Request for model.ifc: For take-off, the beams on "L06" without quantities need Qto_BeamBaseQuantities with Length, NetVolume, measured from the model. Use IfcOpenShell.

First a look at what the model holds.

```python
import ifcopenshell
import ifcopenshell.util.element
import ifcopenshell.util.unit

model = ifcopenshell.open("model.ifc")
print(model.schema)
for unit_type in ("LENGTHUNIT", "AREAUNIT", "VOLUMEUNIT"):
    print(unit_type, ifcopenshell.util.unit.calculate_unit_scale(model, unit_type))
storey = next(s for s in model.by_type("IfcBuildingStorey") if s.Name == "L06")
beams = [e for e in ifcopenshell.util.element.get_decomposition(storey) if e.is_a("IfcBeam")]
for e in sorted(beams, key=lambda e: e.id()):
    print(e.id(), e.is_a(), e.Name, list(ifcopenshell.util.element.get_psets(e, qtos_only=True)), sep=" | ")
```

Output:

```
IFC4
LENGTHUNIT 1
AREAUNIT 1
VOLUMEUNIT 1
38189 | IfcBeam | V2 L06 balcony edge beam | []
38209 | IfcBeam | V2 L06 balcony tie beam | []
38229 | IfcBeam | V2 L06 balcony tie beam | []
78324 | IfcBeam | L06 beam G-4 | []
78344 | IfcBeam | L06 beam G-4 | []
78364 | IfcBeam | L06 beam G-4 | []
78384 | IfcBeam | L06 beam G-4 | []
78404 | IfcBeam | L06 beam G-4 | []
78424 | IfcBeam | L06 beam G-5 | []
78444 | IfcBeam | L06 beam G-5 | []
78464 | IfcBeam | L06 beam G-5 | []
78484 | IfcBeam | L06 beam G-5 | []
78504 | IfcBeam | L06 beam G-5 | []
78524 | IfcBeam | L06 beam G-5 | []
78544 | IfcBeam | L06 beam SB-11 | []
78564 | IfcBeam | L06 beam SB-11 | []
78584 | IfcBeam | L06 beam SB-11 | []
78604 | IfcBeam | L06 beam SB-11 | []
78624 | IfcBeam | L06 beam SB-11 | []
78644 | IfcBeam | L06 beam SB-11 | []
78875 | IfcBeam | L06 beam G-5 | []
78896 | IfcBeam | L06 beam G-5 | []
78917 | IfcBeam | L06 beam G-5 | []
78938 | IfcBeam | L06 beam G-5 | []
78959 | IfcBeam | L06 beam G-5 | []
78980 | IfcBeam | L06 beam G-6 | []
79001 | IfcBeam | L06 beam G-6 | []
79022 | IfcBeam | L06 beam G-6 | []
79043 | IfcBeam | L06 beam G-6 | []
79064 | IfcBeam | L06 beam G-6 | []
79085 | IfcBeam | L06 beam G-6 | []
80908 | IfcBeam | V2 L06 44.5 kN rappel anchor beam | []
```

```python
import ifcopenshell
import ifcopenshell.api.pset
import ifcopenshell.geom
import ifcopenshell.util.element
import ifcopenshell.util.shape
import ifcopenshell.util.unit

model = ifcopenshell.open("model.ifc")
unit_scale = ifcopenshell.util.unit.calculate_unit_scale(model)
volume_scale = ifcopenshell.util.unit.calculate_unit_scale(model, "VOLUMEUNIT")
settings = ifcopenshell.geom.settings()

storey = next(s for s in model.by_type("IfcBuildingStorey") if s.Name == "L06")
beams = [e for e in ifcopenshell.util.element.get_decomposition(storey) if e.is_a("IfcBeam")]

for e in sorted(beams, key=lambda e: e.id()):
    if ifcopenshell.util.element.get_psets(e, qtos_only=True, should_inherit=False):
        continue
    # Geometry comes back in metres, in the element's own axes.
    shape = ifcopenshell.geom.create_shape(settings, e)
    values = {
        "Length": ifcopenshell.util.shape.get_max_xyz(shape.geometry) / unit_scale,
        "NetVolume": ifcopenshell.util.shape.get_volume(shape.geometry) / volume_scale,
    }
    qto = ifcopenshell.api.pset.add_qto(model, product=e, name="Qto_BeamBaseQuantities")
    ifcopenshell.api.pset.edit_qto(model, qto=qto, properties=values)
    print(e.id(), {k: round(v, 3) for k, v in values.items()})

model.write("model-out.ifc")
```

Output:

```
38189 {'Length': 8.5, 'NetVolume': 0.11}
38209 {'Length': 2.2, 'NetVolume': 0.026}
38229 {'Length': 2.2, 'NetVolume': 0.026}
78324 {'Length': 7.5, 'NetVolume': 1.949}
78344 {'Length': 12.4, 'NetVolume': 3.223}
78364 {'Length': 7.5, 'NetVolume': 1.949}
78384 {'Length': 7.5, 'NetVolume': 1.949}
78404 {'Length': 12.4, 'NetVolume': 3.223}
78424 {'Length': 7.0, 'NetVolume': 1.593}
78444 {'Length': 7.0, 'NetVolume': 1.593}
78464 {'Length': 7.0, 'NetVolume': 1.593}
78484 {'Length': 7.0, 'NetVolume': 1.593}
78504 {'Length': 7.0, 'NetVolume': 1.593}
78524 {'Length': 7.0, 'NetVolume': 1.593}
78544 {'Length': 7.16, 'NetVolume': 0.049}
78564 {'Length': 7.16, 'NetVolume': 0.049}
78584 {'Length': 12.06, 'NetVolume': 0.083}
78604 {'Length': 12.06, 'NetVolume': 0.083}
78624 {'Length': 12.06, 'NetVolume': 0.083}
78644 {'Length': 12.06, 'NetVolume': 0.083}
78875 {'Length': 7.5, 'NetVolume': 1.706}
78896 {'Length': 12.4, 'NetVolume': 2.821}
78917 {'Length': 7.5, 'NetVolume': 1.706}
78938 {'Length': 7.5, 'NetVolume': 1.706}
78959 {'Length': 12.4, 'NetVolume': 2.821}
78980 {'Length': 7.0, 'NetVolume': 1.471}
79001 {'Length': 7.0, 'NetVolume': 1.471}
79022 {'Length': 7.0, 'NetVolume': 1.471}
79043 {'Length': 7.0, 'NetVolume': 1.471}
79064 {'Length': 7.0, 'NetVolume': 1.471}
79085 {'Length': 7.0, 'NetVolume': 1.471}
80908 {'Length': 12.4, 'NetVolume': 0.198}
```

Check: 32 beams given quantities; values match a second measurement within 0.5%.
